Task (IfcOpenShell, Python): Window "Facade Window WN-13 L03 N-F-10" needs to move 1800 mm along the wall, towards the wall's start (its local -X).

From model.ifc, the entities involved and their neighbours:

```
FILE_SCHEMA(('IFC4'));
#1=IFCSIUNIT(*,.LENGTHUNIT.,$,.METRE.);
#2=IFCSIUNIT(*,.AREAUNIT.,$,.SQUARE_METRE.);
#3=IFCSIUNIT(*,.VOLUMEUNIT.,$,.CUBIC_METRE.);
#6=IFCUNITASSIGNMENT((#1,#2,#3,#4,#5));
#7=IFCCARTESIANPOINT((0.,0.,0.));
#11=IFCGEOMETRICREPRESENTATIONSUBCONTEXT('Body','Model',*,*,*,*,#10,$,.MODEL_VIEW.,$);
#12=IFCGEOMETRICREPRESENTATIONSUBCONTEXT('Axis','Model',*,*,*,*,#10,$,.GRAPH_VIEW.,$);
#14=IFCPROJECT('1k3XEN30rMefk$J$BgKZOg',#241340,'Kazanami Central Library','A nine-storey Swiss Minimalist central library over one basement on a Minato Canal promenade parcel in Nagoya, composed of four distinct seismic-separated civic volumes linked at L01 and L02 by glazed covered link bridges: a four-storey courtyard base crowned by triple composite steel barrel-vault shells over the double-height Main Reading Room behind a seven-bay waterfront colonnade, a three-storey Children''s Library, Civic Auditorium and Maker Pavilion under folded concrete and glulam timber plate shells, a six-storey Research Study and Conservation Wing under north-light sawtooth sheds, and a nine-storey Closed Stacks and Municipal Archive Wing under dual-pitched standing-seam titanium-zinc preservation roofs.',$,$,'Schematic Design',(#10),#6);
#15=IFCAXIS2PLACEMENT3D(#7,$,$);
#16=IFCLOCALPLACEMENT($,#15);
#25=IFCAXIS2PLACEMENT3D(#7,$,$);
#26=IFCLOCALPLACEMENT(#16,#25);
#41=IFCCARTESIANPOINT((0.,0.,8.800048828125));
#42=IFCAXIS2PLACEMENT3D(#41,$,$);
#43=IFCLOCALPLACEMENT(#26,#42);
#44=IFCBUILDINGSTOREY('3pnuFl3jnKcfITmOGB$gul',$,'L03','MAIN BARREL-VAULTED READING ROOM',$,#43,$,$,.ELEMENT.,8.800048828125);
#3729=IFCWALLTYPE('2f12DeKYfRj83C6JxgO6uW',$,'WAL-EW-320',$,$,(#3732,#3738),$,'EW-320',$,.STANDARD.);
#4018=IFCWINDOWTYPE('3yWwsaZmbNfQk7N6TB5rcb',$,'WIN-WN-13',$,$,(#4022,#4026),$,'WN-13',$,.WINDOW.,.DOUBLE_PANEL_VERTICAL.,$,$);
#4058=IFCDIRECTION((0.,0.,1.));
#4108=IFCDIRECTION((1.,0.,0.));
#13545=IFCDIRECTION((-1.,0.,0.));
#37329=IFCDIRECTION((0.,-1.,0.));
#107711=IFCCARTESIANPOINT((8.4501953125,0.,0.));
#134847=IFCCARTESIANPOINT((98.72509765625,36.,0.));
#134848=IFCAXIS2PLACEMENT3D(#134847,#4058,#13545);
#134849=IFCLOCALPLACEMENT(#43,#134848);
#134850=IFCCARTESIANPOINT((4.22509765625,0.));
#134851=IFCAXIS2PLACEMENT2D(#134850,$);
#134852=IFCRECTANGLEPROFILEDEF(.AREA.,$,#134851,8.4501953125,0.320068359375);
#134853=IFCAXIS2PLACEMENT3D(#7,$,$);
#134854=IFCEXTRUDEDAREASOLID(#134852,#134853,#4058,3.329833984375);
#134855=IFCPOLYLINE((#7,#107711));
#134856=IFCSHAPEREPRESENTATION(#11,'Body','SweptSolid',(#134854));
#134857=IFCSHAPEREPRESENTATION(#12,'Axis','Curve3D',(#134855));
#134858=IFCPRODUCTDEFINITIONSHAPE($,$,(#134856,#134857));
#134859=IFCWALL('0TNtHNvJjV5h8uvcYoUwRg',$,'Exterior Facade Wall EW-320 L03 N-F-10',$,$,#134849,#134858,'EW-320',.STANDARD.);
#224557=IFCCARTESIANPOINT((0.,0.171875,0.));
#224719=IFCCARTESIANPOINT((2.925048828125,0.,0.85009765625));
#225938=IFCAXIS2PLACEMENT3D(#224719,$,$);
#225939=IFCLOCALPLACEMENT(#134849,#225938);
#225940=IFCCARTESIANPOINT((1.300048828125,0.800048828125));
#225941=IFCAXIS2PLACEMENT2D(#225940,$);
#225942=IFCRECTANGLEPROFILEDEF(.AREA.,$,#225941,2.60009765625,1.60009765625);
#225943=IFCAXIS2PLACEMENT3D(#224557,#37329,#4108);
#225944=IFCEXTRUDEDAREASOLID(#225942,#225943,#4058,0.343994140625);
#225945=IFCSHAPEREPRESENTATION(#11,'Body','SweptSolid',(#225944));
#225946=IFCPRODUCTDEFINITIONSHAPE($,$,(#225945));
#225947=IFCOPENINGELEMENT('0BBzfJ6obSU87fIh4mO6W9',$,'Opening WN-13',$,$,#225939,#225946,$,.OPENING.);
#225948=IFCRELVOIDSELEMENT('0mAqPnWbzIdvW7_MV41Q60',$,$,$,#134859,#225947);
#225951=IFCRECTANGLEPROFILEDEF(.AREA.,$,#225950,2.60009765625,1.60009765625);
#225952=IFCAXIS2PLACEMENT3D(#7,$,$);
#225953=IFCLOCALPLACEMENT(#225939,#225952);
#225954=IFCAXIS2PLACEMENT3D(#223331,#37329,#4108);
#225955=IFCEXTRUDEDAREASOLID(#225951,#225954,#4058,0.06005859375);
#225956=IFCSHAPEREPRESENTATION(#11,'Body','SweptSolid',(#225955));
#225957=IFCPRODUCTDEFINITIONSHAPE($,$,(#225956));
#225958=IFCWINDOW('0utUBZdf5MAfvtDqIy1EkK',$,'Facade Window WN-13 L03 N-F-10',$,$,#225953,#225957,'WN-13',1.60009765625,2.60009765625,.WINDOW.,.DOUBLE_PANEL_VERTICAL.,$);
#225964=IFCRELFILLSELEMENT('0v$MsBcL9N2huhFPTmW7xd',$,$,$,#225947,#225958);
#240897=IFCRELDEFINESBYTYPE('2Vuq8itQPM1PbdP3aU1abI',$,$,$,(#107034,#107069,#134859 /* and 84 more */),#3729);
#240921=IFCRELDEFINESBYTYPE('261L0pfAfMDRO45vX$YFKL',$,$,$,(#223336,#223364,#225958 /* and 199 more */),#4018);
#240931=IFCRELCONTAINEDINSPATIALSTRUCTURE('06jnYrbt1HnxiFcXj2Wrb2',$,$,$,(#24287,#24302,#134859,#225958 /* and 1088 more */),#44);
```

```python
import ifcopenshell
import ifcopenshell.api.geometry
import ifcopenshell.util.placement
import ifcopenshell.util.unit

model = ifcopenshell.open("model.ifc")
unit_scale = ifcopenshell.util.unit.calculate_unit_scale(model)

window = model.by_id(225958)
opening = window.FillsVoids[0].RelatingOpeningElement
wall = opening.VoidsElements[0].RelatingBuildingElement

wall_matrix = ifcopenshell.util.placement.get_local_placement(wall.ObjectPlacement)
shift = wall_matrix[:3, 0] * -1.8 / unit_scale
before = ifcopenshell.util.placement.get_local_placement(window.ObjectPlacement)[:3, 3].copy()

# The window is placed relative to its opening, so it follows when the opening moves.
matrix = ifcopenshell.util.placement.get_local_placement(opening.ObjectPlacement)
matrix[:3, 3] += shift
ifcopenshell.api.geometry.edit_object_placement(
    model, product=opening, matrix=matrix, is_si=False, should_transform_children=True
)

after = ifcopenshell.util.placement.get_local_placement(window.ObjectPlacement)[:3, 3]
print("window moved by", (after - before).round(3) + 0.0)

model.write("model-out.ifc")
```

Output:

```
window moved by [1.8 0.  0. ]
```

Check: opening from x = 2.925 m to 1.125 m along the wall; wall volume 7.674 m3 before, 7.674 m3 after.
